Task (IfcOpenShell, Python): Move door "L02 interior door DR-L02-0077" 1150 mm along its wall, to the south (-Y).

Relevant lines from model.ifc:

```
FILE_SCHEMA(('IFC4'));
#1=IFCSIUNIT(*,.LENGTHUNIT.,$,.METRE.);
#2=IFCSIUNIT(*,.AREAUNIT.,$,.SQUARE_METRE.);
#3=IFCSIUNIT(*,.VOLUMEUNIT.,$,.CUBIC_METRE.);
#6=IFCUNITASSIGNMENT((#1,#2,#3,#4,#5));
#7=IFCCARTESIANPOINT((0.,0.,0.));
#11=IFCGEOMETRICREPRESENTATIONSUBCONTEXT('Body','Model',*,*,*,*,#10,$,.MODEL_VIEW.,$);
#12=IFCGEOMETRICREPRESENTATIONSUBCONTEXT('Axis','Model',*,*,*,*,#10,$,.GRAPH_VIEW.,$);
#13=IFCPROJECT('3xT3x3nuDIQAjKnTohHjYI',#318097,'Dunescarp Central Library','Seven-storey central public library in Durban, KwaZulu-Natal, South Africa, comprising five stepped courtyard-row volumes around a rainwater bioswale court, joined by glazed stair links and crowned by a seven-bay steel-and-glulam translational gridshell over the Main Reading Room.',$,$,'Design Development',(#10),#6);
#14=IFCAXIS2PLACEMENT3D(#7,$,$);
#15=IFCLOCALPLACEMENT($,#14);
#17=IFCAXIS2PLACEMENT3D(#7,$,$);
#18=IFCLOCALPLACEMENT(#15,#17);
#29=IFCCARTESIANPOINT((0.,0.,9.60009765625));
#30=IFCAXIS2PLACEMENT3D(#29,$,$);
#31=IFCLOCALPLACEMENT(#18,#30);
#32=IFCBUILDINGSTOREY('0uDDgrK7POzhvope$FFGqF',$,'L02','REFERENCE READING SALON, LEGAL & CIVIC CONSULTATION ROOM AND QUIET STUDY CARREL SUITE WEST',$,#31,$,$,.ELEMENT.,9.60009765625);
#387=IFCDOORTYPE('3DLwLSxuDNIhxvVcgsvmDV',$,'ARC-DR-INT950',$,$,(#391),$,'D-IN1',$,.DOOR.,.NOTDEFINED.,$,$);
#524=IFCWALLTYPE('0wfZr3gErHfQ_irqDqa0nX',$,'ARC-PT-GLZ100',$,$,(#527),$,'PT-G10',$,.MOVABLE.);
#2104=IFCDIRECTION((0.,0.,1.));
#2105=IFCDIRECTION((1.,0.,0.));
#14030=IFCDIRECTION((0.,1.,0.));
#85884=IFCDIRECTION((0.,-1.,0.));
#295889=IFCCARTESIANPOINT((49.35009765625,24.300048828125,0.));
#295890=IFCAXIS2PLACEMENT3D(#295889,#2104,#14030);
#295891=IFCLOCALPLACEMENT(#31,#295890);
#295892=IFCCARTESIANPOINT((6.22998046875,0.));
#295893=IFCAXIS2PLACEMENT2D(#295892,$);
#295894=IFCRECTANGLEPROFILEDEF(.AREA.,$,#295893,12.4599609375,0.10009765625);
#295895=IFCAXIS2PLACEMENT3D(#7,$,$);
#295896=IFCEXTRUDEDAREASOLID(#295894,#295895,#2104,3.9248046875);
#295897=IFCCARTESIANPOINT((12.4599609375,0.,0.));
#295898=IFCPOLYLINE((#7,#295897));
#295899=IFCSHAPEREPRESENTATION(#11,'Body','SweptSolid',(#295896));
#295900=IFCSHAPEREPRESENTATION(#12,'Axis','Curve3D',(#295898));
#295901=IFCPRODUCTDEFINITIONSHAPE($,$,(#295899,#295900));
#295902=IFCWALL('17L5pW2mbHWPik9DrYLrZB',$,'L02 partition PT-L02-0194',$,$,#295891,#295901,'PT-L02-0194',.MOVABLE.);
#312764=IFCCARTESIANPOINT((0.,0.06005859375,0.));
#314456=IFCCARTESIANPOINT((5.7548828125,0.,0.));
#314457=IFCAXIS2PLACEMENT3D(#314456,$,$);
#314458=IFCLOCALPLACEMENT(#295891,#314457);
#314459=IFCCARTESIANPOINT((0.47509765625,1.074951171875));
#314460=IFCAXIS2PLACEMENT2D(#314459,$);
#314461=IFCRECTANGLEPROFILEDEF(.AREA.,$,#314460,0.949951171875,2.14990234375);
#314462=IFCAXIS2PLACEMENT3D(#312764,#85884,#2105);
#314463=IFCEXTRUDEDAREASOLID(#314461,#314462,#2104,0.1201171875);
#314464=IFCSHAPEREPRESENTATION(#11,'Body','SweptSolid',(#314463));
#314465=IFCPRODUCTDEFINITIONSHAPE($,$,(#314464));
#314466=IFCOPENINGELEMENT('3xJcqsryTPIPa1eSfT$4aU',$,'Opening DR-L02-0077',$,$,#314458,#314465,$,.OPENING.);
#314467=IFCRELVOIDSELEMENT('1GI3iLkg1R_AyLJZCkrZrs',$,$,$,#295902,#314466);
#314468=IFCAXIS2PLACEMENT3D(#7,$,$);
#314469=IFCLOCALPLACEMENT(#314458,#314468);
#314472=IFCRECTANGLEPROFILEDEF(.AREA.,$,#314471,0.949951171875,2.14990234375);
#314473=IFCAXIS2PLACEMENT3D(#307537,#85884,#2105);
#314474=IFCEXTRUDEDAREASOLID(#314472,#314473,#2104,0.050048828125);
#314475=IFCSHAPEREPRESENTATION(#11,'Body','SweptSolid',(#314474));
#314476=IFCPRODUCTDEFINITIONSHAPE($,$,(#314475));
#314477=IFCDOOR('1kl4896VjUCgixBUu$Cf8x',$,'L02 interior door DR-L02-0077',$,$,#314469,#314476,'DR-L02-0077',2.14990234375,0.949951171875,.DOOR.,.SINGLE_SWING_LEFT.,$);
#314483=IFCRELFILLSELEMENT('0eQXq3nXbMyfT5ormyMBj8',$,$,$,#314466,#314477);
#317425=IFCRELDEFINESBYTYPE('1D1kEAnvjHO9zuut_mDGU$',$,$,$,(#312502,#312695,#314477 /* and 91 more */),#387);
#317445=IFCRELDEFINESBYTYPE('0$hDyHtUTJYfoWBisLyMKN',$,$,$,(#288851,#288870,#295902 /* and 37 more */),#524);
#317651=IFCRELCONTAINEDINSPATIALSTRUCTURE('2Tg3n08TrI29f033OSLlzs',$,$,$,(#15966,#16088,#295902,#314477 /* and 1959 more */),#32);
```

```python
import ifcopenshell
import ifcopenshell.api.geometry
import ifcopenshell.util.placement

model = ifcopenshell.open("model.ifc")

door = model.by_guid("1kl4896VjUCgixBUu$Cf8x")
opening = door.FillsVoids[0].RelatingOpeningElement
wall = opening.VoidsElements[0].RelatingBuildingElement

wall_matrix = ifcopenshell.util.placement.get_local_placement(wall.ObjectPlacement)
shift = wall_matrix[:3, 0] * -1.15
before = ifcopenshell.util.placement.get_local_placement(door.ObjectPlacement)[:3, 3].copy()

# The door is placed relative to its opening, so it follows when the opening moves.
matrix = ifcopenshell.util.placement.get_local_placement(opening.ObjectPlacement)
matrix[:3, 3] += shift
ifcopenshell.api.geometry.edit_object_placement(
    model, product=opening, matrix=matrix, is_si=False, should_transform_children=True
)

after = ifcopenshell.util.placement.get_local_placement(door.ObjectPlacement)[:3, 3]
print("door moved by", (after - before).round(3) + 0.0)

model.write("model_v2.ifc")
```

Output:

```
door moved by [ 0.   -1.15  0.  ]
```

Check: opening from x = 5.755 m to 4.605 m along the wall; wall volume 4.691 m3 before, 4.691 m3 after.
